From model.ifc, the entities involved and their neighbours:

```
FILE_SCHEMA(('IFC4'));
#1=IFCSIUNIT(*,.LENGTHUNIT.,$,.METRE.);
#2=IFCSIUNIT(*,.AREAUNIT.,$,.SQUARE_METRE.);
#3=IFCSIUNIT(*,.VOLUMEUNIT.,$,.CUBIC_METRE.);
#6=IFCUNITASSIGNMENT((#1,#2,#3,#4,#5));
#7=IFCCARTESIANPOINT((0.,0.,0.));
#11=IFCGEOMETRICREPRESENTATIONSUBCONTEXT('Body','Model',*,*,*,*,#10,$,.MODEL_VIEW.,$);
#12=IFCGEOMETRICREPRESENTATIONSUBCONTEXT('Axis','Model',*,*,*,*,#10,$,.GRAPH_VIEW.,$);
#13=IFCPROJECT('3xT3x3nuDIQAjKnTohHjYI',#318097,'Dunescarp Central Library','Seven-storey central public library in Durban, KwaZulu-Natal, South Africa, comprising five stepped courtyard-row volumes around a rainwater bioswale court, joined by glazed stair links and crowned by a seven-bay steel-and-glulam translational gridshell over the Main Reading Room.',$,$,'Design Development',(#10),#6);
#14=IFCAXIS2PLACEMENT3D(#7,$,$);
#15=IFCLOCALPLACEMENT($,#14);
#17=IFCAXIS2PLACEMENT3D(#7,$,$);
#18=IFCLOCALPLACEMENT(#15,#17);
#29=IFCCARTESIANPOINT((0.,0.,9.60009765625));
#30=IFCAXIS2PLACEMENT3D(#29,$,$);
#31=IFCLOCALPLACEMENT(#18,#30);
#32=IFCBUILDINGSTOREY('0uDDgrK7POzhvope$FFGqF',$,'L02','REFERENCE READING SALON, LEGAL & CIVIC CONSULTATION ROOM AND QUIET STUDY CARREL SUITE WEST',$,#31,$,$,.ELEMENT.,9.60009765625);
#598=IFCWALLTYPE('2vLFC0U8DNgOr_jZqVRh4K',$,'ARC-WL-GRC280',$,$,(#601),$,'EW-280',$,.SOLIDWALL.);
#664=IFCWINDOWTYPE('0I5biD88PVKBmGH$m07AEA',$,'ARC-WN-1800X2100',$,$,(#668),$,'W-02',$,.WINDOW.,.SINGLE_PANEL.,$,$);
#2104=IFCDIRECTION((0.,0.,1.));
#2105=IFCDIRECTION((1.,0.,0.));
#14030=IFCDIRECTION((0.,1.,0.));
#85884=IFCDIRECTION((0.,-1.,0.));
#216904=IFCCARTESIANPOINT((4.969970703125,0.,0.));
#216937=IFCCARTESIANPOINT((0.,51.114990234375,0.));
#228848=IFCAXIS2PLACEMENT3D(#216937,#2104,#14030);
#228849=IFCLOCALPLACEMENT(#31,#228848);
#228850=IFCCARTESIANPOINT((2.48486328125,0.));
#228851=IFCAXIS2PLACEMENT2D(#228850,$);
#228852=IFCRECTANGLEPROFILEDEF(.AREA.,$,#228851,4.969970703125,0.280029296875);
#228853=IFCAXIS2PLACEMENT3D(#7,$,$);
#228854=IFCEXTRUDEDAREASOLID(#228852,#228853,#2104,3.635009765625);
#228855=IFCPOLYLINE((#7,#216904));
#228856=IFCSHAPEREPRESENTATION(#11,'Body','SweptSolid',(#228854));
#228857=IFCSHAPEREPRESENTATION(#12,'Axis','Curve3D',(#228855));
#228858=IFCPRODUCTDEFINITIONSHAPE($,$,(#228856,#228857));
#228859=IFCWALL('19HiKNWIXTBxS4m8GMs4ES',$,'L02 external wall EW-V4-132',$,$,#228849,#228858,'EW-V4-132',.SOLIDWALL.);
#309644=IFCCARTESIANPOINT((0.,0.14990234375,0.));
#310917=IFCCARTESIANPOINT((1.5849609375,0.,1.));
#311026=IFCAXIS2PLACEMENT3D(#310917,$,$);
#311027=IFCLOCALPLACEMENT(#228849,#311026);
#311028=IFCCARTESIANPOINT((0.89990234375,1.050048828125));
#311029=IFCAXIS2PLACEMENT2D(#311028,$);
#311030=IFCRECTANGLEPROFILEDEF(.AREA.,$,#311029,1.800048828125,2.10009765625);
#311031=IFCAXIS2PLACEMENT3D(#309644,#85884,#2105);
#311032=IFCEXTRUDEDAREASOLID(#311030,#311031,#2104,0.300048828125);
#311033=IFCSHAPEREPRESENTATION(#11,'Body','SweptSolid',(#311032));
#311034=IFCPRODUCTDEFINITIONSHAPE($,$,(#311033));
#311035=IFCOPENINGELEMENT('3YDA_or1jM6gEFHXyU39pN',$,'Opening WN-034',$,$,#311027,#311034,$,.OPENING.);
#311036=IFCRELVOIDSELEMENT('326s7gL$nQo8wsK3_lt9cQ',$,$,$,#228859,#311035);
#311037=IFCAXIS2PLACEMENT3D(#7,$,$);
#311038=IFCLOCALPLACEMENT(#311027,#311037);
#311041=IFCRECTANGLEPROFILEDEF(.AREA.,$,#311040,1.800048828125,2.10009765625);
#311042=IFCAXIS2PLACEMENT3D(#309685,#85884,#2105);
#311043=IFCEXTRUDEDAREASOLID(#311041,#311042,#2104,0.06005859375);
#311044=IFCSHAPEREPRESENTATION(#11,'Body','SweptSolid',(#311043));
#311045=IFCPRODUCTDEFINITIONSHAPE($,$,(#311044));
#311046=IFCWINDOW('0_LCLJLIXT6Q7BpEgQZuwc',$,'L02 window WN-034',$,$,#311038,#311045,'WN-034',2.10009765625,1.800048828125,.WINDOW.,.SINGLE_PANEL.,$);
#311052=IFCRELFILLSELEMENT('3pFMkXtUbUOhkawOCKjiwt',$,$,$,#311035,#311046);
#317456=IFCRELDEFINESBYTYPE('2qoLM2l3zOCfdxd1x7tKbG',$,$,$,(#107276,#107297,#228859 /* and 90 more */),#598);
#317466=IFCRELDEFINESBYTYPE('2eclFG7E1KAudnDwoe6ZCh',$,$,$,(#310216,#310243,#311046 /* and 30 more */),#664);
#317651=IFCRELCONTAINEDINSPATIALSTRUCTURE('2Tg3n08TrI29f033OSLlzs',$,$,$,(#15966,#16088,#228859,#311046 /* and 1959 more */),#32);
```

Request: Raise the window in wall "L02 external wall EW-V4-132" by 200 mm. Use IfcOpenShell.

```python
import numpy as np
import ifcopenshell
import ifcopenshell.api.geometry
import ifcopenshell.util.placement
import ifcopenshell.util.unit

model = ifcopenshell.open("model.ifc")
unit_scale = ifcopenshell.util.unit.calculate_unit_scale(model)

window = model.by_guid("0_LCLJLIXT6Q7BpEgQZuwc")
opening = window.FillsVoids[0].RelatingOpeningElement
dz = 0.2 / unit_scale

shift = np.array([0.0, 0.0, dz])
# The window is placed relative to its opening, so it follows when the opening moves.
matrix = ifcopenshell.util.placement.get_local_placement(opening.ObjectPlacement)
matrix[:3, 3] += shift
ifcopenshell.api.geometry.edit_object_placement(
    model, product=opening, matrix=matrix, is_si=False, should_transform_children=True
)

print(f"moved by {dz * unit_scale:+.3f} m")

model.write("model_edited.ifc")
```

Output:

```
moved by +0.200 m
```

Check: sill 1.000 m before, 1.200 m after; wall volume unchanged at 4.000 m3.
